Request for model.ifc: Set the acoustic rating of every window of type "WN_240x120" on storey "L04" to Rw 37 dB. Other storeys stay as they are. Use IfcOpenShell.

First a look at what the model holds.

```python
import ifcopenshell
import ifcopenshell.util.element

model = ifcopenshell.open("model.ifc")
print(model.schema)
storey = next(s for s in model.by_type("IfcBuildingStorey") if s.Name == "L04")
windows = [e for e in ifcopenshell.util.element.get_decomposition(storey) if e.is_a("IfcWindow")]
seen = {}
for e in windows:
    element_type = ifcopenshell.util.element.get_type(e)
    key = (element_type.Name if element_type != e and element_type else None, ifcopenshell.util.element.get_pset(e, "Pset_WindowCommon", "AcousticRating"))
    seen[key] = seen.get(key, 0) + 1
for (name, value), count in sorted(seen.items(), key=str):
    print(count, "x", name, "|", value)
```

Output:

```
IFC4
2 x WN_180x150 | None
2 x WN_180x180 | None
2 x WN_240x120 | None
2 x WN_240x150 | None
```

```python
import ifcopenshell
import ifcopenshell.api.pset
import ifcopenshell.util.element

model = ifcopenshell.open("model.ifc")

storey = next(s for s in model.by_type("IfcBuildingStorey") if s.Name == "L04")
windows = [e for e in ifcopenshell.util.element.get_decomposition(storey) if e.is_a("IfcWindow")]

count = 0
for e in windows:
    element_type = ifcopenshell.util.element.get_type(e)
    if element_type in (None, e) or element_type.Name != "WN_240x120":
        continue
    # add_pset returns the element's existing set when there is one.
    pset = ifcopenshell.api.pset.add_pset(model, product=e, name="Pset_WindowCommon")
    ifcopenshell.api.pset.edit_pset(model, pset=pset, properties={"AcousticRating": "Rw 37 dB"})
    count += 1

print(count, "windows updated")

model.write("model_rev.ifc")
```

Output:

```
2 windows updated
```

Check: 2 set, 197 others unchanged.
